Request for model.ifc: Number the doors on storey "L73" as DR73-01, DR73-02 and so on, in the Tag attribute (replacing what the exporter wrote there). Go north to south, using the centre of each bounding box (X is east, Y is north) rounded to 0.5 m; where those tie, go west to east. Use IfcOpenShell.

First a look at what the model holds.

```python
import ifcopenshell
import ifcopenshell.util.element
import ifcopenshell.util.placement

model = ifcopenshell.open("model.ifc")
print(model.schema)
storey = next(s for s in model.by_type("IfcBuildingStorey") if s.Name == "L73")
doors = [e for e in ifcopenshell.util.element.get_decomposition(storey) if e.is_a("IfcDoor")]
for e in sorted(doors, key=lambda e: e.id()):
    origin = ifcopenshell.util.placement.get_local_placement(e.ObjectPlacement)[:3, 3]
    print(e.id(), e.Tag, e.Name, origin.round(2) + 0.0, sep=" | ")
```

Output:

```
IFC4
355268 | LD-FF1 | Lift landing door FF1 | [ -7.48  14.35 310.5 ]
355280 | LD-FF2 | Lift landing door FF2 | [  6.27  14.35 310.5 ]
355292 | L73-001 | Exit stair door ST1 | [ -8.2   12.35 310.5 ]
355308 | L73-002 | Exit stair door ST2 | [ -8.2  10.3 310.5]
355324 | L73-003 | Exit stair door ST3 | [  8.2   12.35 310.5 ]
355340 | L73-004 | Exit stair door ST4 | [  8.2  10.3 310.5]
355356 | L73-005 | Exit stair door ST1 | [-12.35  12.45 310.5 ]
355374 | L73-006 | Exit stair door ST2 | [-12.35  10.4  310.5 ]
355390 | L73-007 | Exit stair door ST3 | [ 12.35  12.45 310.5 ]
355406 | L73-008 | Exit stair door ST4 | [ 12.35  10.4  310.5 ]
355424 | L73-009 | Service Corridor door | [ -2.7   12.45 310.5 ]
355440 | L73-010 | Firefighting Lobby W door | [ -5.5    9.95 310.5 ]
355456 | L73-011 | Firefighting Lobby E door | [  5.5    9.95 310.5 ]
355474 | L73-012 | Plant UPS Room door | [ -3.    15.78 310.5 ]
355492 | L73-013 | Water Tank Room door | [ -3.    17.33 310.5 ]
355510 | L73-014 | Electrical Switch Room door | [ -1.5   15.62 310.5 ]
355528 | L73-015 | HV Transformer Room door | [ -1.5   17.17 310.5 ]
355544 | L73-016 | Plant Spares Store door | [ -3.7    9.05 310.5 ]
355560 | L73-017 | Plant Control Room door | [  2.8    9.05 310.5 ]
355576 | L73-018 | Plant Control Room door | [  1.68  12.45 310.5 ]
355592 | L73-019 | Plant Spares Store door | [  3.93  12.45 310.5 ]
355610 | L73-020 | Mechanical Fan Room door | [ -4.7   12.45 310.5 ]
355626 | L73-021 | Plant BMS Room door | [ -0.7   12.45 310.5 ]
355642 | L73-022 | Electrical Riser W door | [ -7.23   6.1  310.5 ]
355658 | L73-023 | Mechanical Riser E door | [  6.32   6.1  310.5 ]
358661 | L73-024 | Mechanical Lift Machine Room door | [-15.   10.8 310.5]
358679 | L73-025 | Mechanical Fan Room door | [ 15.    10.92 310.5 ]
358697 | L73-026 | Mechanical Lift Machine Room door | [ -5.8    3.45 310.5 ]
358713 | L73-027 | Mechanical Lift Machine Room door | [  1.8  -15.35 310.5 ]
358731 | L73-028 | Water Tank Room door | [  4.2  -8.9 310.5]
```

```python
import ifcopenshell
import ifcopenshell.geom
import ifcopenshell.util.element
import ifcopenshell.util.shape

model = ifcopenshell.open("model.ifc")
settings = ifcopenshell.geom.settings()
settings.set("use-world-coords", True)


def centre(element):
    shape = ifcopenshell.geom.create_shape(settings, element)
    return ifcopenshell.util.shape.get_bbox_centroid(shape.geometry)


storey = next(s for s in model.by_type("IfcBuildingStorey") if s.Name == "L73")
doors = [e for e in ifcopenshell.util.element.get_decomposition(storey) if e.is_a("IfcDoor")]

# Insertion points can sit at a corner or the storey origin, so sort by the geometry (in metres).
centres = {e: centre(e) for e in doors}
doors.sort(key=lambda e: (-round(centres[e][1] / 0.5), centres[e][0]))

for i, e in enumerate(doors, start=1):
    number = f"DR73-{i:02d}"
    e.Tag = number
    print(e.id(), number)

model.write("model_edited.ifc")
```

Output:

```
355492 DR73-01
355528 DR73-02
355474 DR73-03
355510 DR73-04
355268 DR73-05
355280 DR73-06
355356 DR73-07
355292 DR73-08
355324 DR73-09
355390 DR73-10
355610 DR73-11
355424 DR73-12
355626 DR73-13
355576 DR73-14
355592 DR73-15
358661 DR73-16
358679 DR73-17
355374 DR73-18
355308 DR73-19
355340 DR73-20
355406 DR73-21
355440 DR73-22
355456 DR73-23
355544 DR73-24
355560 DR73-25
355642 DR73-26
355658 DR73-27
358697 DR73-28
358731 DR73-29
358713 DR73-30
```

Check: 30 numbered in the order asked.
